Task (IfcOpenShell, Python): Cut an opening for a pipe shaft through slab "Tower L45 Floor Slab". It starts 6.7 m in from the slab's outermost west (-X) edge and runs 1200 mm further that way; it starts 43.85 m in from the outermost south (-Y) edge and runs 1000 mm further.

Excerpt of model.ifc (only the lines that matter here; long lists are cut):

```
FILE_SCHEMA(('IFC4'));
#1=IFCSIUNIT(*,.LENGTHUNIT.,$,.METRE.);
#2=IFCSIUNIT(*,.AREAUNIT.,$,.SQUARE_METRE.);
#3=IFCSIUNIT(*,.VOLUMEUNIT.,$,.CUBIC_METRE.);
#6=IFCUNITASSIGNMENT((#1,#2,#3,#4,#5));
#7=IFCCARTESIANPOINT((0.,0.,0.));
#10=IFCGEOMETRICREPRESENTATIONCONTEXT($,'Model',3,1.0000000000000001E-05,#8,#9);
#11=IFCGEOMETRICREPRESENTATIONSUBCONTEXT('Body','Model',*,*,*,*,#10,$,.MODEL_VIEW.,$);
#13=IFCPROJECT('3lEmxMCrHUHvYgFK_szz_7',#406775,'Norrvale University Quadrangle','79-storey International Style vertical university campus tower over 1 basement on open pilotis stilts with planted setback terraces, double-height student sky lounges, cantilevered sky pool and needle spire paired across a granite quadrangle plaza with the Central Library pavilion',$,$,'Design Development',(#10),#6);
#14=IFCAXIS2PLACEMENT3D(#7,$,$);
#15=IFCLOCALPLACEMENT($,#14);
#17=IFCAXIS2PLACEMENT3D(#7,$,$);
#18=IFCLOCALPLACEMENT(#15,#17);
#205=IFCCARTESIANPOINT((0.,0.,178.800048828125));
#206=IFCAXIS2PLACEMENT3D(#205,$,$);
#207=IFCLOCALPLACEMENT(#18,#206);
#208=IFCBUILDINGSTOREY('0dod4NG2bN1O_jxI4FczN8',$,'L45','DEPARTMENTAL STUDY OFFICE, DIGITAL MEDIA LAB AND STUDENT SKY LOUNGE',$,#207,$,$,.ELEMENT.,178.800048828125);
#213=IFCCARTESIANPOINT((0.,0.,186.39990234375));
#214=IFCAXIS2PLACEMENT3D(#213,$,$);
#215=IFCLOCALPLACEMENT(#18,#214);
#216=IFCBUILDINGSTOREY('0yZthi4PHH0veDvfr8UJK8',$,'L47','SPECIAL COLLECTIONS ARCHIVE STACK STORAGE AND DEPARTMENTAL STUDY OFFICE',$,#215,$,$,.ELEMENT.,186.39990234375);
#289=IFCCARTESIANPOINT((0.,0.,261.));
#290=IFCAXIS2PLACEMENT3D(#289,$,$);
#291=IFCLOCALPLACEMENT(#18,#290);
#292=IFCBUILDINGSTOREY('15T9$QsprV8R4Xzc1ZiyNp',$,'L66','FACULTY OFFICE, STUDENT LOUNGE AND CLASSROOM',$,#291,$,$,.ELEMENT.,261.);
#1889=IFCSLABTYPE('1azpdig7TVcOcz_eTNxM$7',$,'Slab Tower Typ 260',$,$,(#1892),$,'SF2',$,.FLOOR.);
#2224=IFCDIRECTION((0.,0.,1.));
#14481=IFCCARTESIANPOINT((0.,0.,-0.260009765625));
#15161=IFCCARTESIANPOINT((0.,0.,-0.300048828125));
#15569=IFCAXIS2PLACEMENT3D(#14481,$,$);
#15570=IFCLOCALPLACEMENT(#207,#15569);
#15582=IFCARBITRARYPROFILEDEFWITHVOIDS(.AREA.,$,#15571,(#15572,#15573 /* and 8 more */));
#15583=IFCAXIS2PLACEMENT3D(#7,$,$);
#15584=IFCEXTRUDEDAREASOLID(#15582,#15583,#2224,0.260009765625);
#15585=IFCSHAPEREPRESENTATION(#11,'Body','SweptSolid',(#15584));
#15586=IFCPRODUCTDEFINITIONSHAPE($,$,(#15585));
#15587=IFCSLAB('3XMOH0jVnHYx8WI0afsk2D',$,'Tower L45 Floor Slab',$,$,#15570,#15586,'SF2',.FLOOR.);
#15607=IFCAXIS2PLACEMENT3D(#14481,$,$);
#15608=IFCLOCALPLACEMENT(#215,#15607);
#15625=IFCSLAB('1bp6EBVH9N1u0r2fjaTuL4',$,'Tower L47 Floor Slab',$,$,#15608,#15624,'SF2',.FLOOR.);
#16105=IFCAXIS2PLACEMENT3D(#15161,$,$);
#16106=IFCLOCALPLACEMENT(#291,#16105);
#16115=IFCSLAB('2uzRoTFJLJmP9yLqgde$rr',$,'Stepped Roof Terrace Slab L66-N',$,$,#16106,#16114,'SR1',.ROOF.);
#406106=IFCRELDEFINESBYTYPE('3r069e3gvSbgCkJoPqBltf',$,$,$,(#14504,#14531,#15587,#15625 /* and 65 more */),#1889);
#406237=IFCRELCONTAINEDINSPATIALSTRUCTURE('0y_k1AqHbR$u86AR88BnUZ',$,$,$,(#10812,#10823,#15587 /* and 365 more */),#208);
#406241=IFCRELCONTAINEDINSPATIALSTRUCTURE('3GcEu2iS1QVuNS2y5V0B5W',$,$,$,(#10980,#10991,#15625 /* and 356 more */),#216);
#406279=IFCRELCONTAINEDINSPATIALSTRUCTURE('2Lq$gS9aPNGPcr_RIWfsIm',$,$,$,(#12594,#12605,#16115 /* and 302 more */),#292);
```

```python
import numpy as np
import ifcopenshell
import ifcopenshell.api.feature
import ifcopenshell.api.geometry
import ifcopenshell.api.root
import ifcopenshell.geom
import ifcopenshell.util.placement
import ifcopenshell.util.representation
import ifcopenshell.util.shape
import ifcopenshell.util.unit

model = ifcopenshell.open("model.ifc")
unit_scale = ifcopenshell.util.unit.calculate_unit_scale(model)
settings = ifcopenshell.geom.settings()


def volume(element):
    """Net volume in cubic metres, openings subtracted."""
    shape = ifcopenshell.geom.create_shape(settings, element)
    return ifcopenshell.util.shape.get_volume(shape.geometry)


slab = model.by_guid("3XMOH0jVnHYx8WI0afsk2D")
before = volume(slab)

# Extent in the slab's own axes, in metres. The edges named are its -X and -Y sides.
slab_shape = ifcopenshell.geom.create_shape(settings, slab)
vertices = ifcopenshell.util.shape.get_vertices(slab_shape.geometry)
x_min, y_min, bottom = vertices.min(axis=0)
top = vertices[:, 2].max()

opening = ifcopenshell.api.root.create_entity(model, ifc_class="IfcOpeningElement", name="Pipe shaft opening", predefined_type="OPENING")
context = ifcopenshell.util.representation.get_context(model, "Model", "Body", "MODEL_VIEW")
width, depth = 1.2, 1
outline = [(0.0, 0.0), (width, 0.0), (width, depth), (0.0, depth), (0.0, 0.0)]
# Overshoot both faces by 50 mm so the cut is clean.
shape = ifcopenshell.api.geometry.add_slab_representation(
    model, context=context, depth=top - bottom + 0.1, polyline=outline
)
ifcopenshell.api.geometry.assign_representation(model, product=opening, representation=shape)

matrix = ifcopenshell.util.placement.get_local_placement(slab.ObjectPlacement)
matrix[:, 3] = matrix @ np.append(np.array([x_min + 6.7, y_min + 43.85, bottom - 0.05]) / unit_scale, 1.0)
ifcopenshell.api.geometry.edit_object_placement(model, product=opening, matrix=matrix, is_si=False)
ifcopenshell.api.feature.add_feature(model, feature=opening, element=slab)

after = volume(slab)

print(f"slab volume {before:.3f} -> {after:.3f} m3")

model.write("model_edited.ifc")
```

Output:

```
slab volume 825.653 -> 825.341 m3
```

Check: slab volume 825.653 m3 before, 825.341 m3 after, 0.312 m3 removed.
